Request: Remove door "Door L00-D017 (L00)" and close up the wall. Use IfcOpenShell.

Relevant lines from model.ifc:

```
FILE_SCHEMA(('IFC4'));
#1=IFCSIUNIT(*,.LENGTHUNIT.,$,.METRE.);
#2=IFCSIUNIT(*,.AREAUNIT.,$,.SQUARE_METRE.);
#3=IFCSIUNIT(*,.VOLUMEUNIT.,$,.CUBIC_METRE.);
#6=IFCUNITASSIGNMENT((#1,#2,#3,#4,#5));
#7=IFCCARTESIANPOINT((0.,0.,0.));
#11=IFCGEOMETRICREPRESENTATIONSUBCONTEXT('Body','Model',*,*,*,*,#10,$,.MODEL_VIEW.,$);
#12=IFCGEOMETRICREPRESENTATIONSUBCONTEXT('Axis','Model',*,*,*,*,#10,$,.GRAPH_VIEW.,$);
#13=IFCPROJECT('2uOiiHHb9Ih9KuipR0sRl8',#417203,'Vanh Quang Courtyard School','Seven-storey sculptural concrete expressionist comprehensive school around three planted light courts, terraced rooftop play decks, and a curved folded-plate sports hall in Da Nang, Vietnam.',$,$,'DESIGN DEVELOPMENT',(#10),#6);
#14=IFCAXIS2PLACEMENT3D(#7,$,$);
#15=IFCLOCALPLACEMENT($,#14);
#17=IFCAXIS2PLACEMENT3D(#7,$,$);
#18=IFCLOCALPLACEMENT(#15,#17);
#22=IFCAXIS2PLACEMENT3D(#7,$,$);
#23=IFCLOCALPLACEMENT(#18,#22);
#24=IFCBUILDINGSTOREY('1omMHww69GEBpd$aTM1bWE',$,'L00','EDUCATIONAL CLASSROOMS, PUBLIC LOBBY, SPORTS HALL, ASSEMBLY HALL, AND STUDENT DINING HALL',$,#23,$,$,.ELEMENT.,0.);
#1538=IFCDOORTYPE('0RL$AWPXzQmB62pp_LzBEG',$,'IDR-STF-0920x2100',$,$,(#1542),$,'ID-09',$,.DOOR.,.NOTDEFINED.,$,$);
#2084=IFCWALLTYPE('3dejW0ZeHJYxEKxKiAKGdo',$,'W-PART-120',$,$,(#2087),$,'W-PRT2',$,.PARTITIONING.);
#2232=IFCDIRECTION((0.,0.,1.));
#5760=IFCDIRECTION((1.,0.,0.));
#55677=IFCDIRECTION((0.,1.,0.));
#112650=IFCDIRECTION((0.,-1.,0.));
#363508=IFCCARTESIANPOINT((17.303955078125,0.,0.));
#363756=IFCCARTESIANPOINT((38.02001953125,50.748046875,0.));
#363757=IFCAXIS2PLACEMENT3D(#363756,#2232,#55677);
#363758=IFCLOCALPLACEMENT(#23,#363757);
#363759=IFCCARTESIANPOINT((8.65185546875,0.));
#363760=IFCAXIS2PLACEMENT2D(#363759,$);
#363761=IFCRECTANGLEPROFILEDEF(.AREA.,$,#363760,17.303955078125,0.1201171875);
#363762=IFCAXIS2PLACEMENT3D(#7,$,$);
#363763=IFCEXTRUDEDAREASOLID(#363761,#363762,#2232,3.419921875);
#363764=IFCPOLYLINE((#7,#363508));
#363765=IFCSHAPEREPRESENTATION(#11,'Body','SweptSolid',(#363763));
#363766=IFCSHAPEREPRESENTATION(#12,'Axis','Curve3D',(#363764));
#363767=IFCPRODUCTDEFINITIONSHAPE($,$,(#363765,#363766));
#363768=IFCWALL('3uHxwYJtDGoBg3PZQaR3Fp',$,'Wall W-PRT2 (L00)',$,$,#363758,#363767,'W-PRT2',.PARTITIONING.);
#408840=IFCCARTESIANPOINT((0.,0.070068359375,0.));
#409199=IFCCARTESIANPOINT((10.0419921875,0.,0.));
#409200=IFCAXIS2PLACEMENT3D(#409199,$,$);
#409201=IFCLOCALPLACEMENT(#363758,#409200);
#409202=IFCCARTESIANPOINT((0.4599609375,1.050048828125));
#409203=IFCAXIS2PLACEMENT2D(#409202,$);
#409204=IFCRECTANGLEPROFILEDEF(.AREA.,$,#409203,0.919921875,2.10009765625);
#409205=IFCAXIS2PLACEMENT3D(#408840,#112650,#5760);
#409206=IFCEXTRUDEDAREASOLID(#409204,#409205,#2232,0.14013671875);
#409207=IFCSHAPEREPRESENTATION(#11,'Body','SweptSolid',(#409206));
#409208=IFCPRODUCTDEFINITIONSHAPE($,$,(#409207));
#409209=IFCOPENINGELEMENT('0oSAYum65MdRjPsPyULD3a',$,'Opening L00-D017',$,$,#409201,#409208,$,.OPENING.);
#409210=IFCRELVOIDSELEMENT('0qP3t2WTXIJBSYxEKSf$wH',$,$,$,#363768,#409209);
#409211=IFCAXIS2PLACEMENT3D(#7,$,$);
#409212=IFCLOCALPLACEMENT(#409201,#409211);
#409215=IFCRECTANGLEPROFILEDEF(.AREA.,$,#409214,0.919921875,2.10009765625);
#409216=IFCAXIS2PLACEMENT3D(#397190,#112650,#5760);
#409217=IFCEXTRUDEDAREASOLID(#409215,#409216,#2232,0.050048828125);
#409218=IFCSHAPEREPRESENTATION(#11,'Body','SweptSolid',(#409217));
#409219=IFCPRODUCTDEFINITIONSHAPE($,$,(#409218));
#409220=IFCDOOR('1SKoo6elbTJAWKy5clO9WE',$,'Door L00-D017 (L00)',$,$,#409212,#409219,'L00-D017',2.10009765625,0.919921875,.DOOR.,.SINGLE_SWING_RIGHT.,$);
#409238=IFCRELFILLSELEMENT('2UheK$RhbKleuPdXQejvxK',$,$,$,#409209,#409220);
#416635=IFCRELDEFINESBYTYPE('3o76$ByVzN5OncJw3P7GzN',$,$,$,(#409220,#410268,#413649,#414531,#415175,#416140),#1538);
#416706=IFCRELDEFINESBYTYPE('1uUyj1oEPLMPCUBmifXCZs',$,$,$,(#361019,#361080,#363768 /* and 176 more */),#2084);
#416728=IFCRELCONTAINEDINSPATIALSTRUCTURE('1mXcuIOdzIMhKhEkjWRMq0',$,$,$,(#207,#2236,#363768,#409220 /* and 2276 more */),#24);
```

```python
import ifcopenshell
import ifcopenshell.api.feature
import ifcopenshell.api.root
import ifcopenshell.geom
import ifcopenshell.util.shape

model = ifcopenshell.open("model.ifc")
settings = ifcopenshell.geom.settings()


def volume(element):
    """Net volume in cubic metres, openings subtracted."""
    shape = ifcopenshell.geom.create_shape(settings, element)
    return ifcopenshell.util.shape.get_volume(shape.geometry)


door = model.by_id(409220)
opening = door.FillsVoids[0].RelatingOpeningElement
wall = opening.VoidsElements[0].RelatingBuildingElement
before = volume(wall)

ifcopenshell.api.root.remove_product(model, product=door)
ifcopenshell.api.feature.remove_feature(model, feature=opening)

after = volume(wall)

print(f"wall volume {before:.3f} -> {after:.3f} m3")

model.write("model_v2.ifc")
```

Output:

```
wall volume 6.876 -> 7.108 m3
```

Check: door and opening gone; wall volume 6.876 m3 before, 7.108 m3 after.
